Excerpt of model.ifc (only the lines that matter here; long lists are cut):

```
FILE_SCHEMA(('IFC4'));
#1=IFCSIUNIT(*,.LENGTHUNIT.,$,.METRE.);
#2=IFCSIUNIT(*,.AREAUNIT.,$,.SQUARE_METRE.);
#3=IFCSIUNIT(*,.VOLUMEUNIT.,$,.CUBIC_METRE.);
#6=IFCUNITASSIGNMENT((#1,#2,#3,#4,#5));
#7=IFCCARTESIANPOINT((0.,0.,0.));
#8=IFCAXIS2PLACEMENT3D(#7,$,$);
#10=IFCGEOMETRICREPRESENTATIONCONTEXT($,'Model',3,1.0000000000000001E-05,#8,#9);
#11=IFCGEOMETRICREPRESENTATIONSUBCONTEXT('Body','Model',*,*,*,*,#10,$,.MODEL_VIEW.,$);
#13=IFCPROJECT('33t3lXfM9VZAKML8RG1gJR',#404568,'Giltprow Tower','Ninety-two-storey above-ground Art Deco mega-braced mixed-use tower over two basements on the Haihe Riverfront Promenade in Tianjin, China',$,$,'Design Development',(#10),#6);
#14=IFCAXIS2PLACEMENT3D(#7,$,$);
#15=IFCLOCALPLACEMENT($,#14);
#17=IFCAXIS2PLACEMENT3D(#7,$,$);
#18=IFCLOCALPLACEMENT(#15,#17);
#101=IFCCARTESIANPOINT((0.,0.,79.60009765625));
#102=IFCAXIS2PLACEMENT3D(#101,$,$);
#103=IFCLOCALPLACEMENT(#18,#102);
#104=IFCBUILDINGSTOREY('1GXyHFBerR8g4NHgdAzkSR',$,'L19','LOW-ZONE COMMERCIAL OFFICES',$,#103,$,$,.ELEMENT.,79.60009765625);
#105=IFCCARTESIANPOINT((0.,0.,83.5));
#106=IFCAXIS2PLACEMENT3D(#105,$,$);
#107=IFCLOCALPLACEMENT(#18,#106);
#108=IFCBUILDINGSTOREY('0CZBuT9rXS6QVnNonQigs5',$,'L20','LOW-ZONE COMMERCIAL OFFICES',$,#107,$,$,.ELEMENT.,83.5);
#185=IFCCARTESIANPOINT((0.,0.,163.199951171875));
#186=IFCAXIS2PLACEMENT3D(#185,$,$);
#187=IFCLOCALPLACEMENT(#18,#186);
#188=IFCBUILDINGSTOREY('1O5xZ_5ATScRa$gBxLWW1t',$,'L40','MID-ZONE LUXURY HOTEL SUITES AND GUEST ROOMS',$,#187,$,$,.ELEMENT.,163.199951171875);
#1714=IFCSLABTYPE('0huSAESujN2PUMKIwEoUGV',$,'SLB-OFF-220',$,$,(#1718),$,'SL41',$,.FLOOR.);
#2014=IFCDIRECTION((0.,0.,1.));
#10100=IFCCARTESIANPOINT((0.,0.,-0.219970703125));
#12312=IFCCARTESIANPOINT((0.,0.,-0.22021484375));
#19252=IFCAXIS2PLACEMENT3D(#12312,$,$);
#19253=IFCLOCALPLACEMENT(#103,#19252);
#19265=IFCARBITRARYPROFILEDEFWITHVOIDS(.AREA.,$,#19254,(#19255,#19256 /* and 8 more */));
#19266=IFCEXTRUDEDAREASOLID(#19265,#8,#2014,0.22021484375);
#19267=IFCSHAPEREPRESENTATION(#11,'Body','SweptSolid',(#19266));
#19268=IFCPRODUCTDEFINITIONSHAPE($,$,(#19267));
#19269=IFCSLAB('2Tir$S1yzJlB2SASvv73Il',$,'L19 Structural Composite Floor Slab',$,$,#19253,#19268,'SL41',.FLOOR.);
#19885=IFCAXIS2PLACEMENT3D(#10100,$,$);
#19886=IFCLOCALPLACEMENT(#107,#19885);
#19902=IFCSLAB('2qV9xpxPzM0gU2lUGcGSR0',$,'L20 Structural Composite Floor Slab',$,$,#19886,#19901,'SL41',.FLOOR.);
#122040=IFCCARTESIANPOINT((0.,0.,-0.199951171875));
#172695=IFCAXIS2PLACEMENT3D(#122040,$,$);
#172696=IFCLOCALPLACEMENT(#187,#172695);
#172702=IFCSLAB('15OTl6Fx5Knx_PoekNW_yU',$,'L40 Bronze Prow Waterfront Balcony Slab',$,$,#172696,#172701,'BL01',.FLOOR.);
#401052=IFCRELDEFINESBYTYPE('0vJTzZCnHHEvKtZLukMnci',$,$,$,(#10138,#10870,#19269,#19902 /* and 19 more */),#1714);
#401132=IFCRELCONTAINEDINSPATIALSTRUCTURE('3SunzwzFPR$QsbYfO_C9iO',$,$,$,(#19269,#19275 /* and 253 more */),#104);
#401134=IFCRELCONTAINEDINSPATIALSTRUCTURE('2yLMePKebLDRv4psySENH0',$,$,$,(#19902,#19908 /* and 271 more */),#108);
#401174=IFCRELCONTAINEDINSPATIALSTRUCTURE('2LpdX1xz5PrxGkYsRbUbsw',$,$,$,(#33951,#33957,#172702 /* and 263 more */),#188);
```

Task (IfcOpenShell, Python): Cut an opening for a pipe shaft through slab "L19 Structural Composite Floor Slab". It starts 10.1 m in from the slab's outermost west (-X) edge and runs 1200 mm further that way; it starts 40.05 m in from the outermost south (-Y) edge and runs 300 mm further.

```python
import numpy as np
import ifcopenshell
import ifcopenshell.api.feature
import ifcopenshell.api.geometry
import ifcopenshell.api.root
import ifcopenshell.geom
import ifcopenshell.util.placement
import ifcopenshell.util.representation
import ifcopenshell.util.shape
import ifcopenshell.util.unit

model = ifcopenshell.open("model.ifc")
unit_scale = ifcopenshell.util.unit.calculate_unit_scale(model)
settings = ifcopenshell.geom.settings()


def volume(element):
    """Net volume in cubic metres, openings subtracted."""
    shape = ifcopenshell.geom.create_shape(settings, element)
    return ifcopenshell.util.shape.get_volume(shape.geometry)


slab = model.by_guid("2Tir$S1yzJlB2SASvv73Il")
before = volume(slab)

# Extent in the slab's own axes, in metres. The edges named are its -X and -Y sides.
slab_shape = ifcopenshell.geom.create_shape(settings, slab)
vertices = ifcopenshell.util.shape.get_vertices(slab_shape.geometry)
x_min, y_min, bottom = vertices.min(axis=0)
top = vertices[:, 2].max()

opening = ifcopenshell.api.root.create_entity(model, ifc_class="IfcOpeningElement", name="Pipe shaft opening", predefined_type="OPENING")
context = ifcopenshell.util.representation.get_context(model, "Model", "Body", "MODEL_VIEW")
width, depth = 1.2, 0.3
outline = [(0.0, 0.0), (width, 0.0), (width, depth), (0.0, depth), (0.0, 0.0)]
# Overshoot both faces by 50 mm so the cut is clean.
shape = ifcopenshell.api.geometry.add_slab_representation(
    model, context=context, depth=top - bottom + 0.1, polyline=outline
)
ifcopenshell.api.geometry.assign_representation(model, product=opening, representation=shape)

matrix = ifcopenshell.util.placement.get_local_placement(slab.ObjectPlacement)
matrix[:, 3] = matrix @ np.append(np.array([x_min + 10.1, y_min + 40.05, bottom - 0.05]) / unit_scale, 1.0)
ifcopenshell.api.geometry.edit_object_placement(model, product=opening, matrix=matrix, is_si=False)
ifcopenshell.api.feature.add_feature(model, feature=opening, element=slab)

after = volume(slab)

print(f"slab volume {before:.3f} -> {after:.3f} m3")

model.write("model_edited.ifc")
```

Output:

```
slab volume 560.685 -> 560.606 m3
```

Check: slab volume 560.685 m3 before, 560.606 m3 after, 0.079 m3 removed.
